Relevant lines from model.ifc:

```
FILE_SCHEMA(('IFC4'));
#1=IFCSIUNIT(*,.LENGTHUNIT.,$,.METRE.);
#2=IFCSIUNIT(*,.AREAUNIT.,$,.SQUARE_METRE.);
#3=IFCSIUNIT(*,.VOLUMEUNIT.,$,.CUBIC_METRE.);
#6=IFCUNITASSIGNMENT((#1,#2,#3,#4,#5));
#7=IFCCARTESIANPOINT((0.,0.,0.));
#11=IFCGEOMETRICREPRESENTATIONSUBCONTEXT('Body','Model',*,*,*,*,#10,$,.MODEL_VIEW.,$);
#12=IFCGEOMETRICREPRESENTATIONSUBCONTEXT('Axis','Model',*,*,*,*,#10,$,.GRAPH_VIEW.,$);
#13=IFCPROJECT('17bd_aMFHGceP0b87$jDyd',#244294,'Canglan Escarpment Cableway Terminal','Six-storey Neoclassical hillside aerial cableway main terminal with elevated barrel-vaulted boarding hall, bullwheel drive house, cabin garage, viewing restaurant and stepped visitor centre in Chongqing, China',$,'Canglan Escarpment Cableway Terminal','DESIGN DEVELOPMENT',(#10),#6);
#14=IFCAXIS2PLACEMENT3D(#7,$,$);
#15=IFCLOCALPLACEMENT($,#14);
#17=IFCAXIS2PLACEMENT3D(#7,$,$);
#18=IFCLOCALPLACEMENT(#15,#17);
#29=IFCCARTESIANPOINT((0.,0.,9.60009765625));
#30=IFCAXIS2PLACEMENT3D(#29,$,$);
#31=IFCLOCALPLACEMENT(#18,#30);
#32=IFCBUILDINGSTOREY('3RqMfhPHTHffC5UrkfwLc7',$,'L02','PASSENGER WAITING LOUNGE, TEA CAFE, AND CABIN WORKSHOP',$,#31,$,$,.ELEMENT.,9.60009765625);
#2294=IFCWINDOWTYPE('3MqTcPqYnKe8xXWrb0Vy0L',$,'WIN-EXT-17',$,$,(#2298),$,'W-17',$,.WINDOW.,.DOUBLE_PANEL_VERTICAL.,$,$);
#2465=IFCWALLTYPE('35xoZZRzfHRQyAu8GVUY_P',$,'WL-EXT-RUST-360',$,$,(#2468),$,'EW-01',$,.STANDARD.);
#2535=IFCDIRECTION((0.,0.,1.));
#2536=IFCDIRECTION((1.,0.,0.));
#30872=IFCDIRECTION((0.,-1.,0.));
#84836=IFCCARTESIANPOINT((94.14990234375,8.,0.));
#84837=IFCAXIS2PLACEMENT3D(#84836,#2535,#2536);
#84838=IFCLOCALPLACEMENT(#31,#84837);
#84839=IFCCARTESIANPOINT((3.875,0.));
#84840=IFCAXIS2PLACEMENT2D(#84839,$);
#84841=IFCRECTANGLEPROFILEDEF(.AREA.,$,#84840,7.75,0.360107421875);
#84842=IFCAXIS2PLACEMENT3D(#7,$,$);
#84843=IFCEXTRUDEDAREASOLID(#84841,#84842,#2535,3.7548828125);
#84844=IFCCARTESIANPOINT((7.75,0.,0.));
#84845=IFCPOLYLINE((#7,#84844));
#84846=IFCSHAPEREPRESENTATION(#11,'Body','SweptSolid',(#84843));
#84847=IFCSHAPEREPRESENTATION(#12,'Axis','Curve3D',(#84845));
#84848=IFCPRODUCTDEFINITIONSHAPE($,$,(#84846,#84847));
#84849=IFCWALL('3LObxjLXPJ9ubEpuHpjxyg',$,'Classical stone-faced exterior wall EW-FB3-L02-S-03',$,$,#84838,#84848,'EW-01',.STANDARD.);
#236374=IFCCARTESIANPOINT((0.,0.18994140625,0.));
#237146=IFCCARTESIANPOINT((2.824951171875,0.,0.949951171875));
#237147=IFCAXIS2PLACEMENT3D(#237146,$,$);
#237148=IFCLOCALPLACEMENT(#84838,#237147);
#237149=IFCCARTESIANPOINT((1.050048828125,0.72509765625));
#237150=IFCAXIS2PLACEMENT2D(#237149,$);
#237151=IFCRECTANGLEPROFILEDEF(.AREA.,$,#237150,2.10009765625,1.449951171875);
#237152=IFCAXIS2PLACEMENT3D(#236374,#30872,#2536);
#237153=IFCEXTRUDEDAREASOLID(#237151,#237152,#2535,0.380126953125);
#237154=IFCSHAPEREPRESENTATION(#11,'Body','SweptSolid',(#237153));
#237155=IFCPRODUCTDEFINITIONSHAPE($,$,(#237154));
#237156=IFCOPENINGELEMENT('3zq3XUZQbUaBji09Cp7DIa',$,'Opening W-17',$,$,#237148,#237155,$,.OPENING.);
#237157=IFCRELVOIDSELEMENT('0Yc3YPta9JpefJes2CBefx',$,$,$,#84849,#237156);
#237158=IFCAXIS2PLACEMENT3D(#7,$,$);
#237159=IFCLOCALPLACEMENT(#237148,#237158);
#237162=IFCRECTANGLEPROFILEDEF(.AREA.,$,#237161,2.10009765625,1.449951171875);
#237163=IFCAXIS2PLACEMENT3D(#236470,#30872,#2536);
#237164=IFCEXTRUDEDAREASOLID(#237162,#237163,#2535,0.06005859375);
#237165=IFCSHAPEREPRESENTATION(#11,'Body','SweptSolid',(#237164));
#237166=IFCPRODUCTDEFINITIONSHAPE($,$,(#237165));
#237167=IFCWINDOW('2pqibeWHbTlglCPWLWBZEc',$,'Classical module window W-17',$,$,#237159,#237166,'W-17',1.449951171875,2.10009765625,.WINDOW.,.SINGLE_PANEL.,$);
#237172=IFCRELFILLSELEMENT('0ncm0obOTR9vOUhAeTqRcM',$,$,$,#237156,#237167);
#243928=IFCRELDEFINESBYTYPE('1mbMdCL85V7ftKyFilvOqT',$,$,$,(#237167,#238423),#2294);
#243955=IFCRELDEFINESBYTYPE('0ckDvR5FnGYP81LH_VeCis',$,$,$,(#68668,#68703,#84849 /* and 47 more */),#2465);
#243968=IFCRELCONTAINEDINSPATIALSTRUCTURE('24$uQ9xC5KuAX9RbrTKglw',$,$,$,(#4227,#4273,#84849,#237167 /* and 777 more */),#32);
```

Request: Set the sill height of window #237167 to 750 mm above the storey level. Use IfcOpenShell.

```python
import numpy as np
import ifcopenshell
import ifcopenshell.api.geometry
import ifcopenshell.geom
import ifcopenshell.util.element
import ifcopenshell.util.placement
import ifcopenshell.util.shape
import ifcopenshell.util.unit

model = ifcopenshell.open("model.ifc")
unit_scale = ifcopenshell.util.unit.calculate_unit_scale(model)

window = model.by_guid("2pqibeWHbTlglCPWLWBZEc")
opening = window.FillsVoids[0].RelatingOpeningElement
storey = ifcopenshell.util.element.get_container(window, ifc_class="IfcBuildingStorey")
level = ifcopenshell.util.placement.get_local_placement(storey.ObjectPlacement)[2, 3]

# The opening's origin need not be at the sill, so measure its lowest point.
shape = ifcopenshell.geom.create_shape(ifcopenshell.geom.settings(), opening)
bottom = ifcopenshell.util.shape.get_shape_bottom_elevation(shape, shape.geometry) / unit_scale
dz = level + 0.75 / unit_scale - bottom

shift = np.array([0.0, 0.0, dz])
# The window is placed relative to its opening, so it follows when the opening moves.
matrix = ifcopenshell.util.placement.get_local_placement(opening.ObjectPlacement)
matrix[:3, 3] += shift
ifcopenshell.api.geometry.edit_object_placement(
    model, product=opening, matrix=matrix, is_si=False, should_transform_children=True
)

print(f"moved by {dz * unit_scale:+.3f} m")

model.write("model-out.ifc")
```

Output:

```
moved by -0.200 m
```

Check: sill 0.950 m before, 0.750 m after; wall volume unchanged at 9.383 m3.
